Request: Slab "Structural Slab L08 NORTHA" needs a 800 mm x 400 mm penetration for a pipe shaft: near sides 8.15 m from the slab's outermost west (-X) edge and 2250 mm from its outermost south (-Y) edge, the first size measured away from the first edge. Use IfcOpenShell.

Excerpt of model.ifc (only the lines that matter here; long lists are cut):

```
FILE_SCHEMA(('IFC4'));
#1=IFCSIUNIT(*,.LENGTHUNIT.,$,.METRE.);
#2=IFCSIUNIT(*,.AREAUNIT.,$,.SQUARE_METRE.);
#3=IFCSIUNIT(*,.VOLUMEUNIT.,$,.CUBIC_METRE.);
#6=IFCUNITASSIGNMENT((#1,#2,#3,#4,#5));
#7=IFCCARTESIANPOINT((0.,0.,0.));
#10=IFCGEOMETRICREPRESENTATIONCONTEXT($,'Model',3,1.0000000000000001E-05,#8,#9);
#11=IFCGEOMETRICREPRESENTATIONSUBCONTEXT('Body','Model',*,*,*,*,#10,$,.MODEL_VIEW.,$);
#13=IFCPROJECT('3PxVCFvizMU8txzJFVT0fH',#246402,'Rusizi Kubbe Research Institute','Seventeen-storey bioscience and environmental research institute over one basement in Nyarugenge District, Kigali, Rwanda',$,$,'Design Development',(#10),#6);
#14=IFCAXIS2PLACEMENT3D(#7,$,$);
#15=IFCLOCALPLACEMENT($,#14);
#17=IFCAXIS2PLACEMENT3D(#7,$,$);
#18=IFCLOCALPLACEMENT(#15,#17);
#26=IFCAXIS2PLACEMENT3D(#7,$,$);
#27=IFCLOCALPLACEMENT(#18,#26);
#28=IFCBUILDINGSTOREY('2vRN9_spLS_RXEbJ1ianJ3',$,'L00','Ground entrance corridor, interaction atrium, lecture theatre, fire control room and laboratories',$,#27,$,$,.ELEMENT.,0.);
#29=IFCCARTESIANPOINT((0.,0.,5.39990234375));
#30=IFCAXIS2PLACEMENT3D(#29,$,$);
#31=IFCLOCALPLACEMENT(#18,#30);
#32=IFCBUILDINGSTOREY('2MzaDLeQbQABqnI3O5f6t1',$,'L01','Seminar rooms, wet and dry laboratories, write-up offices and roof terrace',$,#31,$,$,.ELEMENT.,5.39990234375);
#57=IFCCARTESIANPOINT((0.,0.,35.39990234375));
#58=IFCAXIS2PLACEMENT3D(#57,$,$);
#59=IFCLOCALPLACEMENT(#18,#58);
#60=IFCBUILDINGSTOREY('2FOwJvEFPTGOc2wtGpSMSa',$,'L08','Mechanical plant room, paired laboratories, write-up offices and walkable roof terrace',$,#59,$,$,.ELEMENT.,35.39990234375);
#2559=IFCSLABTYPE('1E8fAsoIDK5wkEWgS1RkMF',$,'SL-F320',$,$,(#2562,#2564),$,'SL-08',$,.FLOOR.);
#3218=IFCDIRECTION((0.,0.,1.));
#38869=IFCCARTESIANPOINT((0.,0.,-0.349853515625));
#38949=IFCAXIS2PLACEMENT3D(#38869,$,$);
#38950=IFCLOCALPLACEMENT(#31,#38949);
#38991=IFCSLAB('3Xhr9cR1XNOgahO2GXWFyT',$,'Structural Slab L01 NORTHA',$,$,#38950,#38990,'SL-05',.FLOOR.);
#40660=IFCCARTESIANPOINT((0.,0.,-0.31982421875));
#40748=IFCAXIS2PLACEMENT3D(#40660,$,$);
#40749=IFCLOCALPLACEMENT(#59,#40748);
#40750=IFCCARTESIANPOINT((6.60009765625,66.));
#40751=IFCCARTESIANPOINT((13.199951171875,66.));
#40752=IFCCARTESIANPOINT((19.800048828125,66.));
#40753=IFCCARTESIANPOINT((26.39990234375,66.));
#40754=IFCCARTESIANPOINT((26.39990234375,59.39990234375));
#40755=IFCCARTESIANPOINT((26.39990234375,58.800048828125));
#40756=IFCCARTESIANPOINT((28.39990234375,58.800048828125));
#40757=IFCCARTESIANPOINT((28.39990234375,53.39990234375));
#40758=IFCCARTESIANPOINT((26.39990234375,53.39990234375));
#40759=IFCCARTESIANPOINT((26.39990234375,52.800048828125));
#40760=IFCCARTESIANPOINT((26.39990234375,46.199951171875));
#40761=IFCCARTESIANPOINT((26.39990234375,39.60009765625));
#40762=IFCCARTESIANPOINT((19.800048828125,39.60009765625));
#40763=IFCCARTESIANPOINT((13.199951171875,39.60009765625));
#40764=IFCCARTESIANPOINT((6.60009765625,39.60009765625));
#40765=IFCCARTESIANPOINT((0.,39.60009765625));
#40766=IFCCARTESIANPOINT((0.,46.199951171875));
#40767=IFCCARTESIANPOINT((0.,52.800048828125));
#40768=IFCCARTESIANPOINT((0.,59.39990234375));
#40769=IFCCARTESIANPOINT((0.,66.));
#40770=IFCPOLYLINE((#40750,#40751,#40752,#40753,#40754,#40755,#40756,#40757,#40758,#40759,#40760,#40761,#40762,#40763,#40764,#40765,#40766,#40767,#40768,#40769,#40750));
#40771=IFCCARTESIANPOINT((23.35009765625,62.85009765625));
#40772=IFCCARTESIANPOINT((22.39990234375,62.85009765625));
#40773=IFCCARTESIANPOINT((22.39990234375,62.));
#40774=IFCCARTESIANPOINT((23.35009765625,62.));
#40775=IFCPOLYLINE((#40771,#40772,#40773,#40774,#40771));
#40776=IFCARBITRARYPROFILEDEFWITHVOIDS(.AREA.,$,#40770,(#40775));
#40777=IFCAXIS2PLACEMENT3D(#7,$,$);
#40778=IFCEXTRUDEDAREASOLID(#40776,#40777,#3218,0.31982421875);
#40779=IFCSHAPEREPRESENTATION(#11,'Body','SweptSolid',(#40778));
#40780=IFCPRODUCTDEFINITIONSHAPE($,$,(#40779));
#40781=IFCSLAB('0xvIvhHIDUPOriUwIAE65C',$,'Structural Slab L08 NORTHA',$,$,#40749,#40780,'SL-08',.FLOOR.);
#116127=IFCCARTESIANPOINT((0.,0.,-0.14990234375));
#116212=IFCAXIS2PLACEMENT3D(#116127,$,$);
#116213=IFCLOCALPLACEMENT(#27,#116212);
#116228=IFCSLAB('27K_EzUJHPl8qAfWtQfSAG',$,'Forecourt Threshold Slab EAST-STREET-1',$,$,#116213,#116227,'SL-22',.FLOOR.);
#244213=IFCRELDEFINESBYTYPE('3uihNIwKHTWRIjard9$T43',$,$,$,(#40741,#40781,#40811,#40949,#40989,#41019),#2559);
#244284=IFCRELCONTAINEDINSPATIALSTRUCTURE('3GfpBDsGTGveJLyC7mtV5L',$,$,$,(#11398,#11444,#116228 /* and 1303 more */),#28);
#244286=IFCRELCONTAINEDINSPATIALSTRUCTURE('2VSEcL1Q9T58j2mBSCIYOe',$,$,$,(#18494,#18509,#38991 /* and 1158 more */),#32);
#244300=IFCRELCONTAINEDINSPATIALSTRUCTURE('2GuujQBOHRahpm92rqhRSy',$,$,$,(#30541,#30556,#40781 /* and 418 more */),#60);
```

```python
import numpy as np
import ifcopenshell
import ifcopenshell.api.feature
import ifcopenshell.api.geometry
import ifcopenshell.api.root
import ifcopenshell.geom
import ifcopenshell.util.placement
import ifcopenshell.util.representation
import ifcopenshell.util.shape
import ifcopenshell.util.unit

model = ifcopenshell.open("model.ifc")
unit_scale = ifcopenshell.util.unit.calculate_unit_scale(model)
settings = ifcopenshell.geom.settings()


def volume(element):
    """Net volume in cubic metres, openings subtracted."""
    shape = ifcopenshell.geom.create_shape(settings, element)
    return ifcopenshell.util.shape.get_volume(shape.geometry)


slab = model.by_id(40781)
before = volume(slab)

# Extent in the slab's own axes, in metres. The edges named are its -X and -Y sides.
slab_shape = ifcopenshell.geom.create_shape(settings, slab)
vertices = ifcopenshell.util.shape.get_vertices(slab_shape.geometry)
x_min, y_min, bottom = vertices.min(axis=0)
top = vertices[:, 2].max()

opening = ifcopenshell.api.root.create_entity(model, ifc_class="IfcOpeningElement", name="Pipe shaft opening", predefined_type="OPENING")
context = ifcopenshell.util.representation.get_context(model, "Model", "Body", "MODEL_VIEW")
width, depth = 0.8, 0.4
outline = [(0.0, 0.0), (width, 0.0), (width, depth), (0.0, depth), (0.0, 0.0)]
# Overshoot both faces by 50 mm so the cut is clean.
shape = ifcopenshell.api.geometry.add_slab_representation(
    model, context=context, depth=top - bottom + 0.1, polyline=outline
)
ifcopenshell.api.geometry.assign_representation(model, product=opening, representation=shape)

matrix = ifcopenshell.util.placement.get_local_placement(slab.ObjectPlacement)
matrix[:, 3] = matrix @ np.append(np.array([x_min + 8.15, y_min + 2.25, bottom - 0.05]) / unit_scale, 1.0)
ifcopenshell.api.geometry.edit_object_placement(model, product=opening, matrix=matrix, is_si=False)
ifcopenshell.api.feature.add_feature(model, feature=opening, element=slab)

after = volume(slab)

print(f"slab volume {before:.3f} -> {after:.3f} m3")

model.write("model_v2.ifc")
```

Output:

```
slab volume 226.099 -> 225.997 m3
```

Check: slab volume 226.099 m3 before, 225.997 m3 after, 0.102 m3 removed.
